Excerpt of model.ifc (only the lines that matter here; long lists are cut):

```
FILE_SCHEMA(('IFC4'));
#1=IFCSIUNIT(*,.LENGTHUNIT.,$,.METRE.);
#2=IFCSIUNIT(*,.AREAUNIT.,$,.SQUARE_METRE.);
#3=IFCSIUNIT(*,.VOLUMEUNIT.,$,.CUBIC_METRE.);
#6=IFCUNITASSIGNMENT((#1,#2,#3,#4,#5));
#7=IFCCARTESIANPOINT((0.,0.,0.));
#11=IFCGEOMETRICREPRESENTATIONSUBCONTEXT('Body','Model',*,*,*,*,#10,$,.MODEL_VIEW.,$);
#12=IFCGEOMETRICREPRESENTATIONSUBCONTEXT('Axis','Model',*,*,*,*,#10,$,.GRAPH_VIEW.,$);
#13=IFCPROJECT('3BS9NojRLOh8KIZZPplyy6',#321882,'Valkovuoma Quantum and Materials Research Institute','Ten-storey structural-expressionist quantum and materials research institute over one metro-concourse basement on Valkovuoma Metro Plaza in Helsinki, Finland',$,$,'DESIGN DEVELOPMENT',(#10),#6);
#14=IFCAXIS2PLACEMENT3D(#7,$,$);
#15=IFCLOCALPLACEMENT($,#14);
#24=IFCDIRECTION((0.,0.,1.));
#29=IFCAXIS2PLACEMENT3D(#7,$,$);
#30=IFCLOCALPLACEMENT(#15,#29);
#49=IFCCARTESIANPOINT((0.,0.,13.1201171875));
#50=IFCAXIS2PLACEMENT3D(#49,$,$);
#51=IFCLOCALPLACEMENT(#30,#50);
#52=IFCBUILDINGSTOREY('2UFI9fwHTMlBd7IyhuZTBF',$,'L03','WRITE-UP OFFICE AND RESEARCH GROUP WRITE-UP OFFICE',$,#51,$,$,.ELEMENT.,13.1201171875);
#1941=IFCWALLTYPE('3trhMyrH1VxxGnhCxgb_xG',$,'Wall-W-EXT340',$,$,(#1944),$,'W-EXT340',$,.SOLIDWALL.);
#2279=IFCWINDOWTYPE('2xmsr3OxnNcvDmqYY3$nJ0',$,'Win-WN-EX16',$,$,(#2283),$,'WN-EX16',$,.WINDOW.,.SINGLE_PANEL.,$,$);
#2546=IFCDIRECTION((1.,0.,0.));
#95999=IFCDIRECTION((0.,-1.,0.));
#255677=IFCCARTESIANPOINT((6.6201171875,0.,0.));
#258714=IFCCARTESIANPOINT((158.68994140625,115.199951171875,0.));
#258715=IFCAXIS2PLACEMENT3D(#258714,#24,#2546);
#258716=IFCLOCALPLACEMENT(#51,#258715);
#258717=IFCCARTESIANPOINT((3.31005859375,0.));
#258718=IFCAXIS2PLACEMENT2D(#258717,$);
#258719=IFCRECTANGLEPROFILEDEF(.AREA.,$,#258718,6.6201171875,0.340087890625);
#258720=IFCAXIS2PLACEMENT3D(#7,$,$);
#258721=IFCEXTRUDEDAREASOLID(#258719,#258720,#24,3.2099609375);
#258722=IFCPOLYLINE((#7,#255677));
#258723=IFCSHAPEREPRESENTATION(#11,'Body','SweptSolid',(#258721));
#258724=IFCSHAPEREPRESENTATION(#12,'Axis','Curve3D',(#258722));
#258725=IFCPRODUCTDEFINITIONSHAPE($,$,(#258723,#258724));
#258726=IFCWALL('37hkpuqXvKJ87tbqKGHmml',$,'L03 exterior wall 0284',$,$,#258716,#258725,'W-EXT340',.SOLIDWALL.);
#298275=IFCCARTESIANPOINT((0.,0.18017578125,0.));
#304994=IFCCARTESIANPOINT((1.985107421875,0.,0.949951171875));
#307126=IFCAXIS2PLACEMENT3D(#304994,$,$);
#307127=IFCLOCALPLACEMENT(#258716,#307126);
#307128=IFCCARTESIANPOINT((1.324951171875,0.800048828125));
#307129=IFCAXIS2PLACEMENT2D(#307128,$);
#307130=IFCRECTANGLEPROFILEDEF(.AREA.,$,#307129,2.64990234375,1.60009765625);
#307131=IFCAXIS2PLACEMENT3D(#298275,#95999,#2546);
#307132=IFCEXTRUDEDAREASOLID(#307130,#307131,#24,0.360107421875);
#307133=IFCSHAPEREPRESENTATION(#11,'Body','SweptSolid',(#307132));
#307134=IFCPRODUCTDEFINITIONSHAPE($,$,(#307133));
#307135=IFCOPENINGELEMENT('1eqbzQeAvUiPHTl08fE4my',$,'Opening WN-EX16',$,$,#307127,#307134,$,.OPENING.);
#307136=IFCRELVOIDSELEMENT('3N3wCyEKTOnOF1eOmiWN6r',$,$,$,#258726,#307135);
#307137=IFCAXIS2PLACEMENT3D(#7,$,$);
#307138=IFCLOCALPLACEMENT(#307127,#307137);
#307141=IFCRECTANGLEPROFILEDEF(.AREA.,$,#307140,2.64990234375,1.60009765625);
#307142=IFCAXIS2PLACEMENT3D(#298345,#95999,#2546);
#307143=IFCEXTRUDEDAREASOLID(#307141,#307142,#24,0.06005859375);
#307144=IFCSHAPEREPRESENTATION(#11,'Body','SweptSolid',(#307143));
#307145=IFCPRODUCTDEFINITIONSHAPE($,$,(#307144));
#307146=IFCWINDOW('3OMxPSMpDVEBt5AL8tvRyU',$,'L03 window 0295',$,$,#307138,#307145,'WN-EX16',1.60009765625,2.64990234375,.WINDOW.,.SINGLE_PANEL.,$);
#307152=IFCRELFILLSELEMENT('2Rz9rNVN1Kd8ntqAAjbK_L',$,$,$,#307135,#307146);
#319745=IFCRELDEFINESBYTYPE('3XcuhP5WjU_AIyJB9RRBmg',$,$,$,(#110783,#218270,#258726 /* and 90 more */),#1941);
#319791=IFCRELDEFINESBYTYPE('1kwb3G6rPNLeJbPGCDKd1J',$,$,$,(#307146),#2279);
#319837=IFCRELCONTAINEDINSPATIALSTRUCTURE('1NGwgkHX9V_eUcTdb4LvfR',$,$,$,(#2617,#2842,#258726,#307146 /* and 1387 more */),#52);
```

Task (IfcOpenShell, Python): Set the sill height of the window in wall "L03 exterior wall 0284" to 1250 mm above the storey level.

```python
import numpy as np
import ifcopenshell
import ifcopenshell.api.geometry
import ifcopenshell.geom
import ifcopenshell.util.element
import ifcopenshell.util.placement
import ifcopenshell.util.shape
import ifcopenshell.util.unit

model = ifcopenshell.open("model.ifc")
unit_scale = ifcopenshell.util.unit.calculate_unit_scale(model)

window = model.by_id(307146)
opening = window.FillsVoids[0].RelatingOpeningElement
storey = ifcopenshell.util.element.get_container(window, ifc_class="IfcBuildingStorey")
level = ifcopenshell.util.placement.get_local_placement(storey.ObjectPlacement)[2, 3]

# The opening's origin need not be at the sill, so measure its lowest point.
shape = ifcopenshell.geom.create_shape(ifcopenshell.geom.settings(), opening)
bottom = ifcopenshell.util.shape.get_shape_bottom_elevation(shape, shape.geometry) / unit_scale
dz = level + 1.25 - bottom

shift = np.array([0.0, 0.0, dz])
# The window is placed relative to its opening, so it follows when the opening moves.
matrix = ifcopenshell.util.placement.get_local_placement(opening.ObjectPlacement)
matrix[:3, 3] += shift
ifcopenshell.api.geometry.edit_object_placement(
    model, product=opening, matrix=matrix, is_si=False, should_transform_children=True
)

print(f"moved by {dz * unit_scale:+.3f} m")

model.write("model_updated.ifc")
```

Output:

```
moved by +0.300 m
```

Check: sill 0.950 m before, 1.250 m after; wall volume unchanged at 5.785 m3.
